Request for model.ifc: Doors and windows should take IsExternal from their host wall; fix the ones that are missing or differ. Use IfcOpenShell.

First a look at what the model holds.

```python
import ifcopenshell
import ifcopenshell.util.element

model = ifcopenshell.open("model.ifc")
print(model.schema)
seen = {}
for e in model.by_type("IfcDoor") + model.by_type("IfcWindow"):
    if not e.FillsVoids:
        continue
    host = e.FillsVoids[0].RelatingOpeningElement.VoidsElements[0].RelatingBuildingElement
    own = ifcopenshell.util.element.get_pset(e, f"Pset_{e.is_a()[3:].removesuffix('StandardCase')}Common", "IsExternal")
    wall = ifcopenshell.util.element.get_pset(host, "Pset_WallCommon", "IsExternal")
    seen[e.is_a(), own, wall] = seen.get((e.is_a(), own, wall), 0) + 1
for (cls, own, wall), count in sorted(seen.items(), key=str):
    print(count, cls, "IsExternal:", own, "| host wall:", wall)
```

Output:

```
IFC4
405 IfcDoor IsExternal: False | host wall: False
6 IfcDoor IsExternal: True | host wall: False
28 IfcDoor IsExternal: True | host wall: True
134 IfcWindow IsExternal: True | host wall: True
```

```python
import ifcopenshell
import ifcopenshell.api.pset
import ifcopenshell.util.element

model = ifcopenshell.open("model.ifc")

count = 0
for ifc_class, pset_name in (("IfcDoor", "Pset_DoorCommon"), ("IfcWindow", "Pset_WindowCommon")):
    for e in model.by_type(ifc_class):
        if not e.FillsVoids:
            continue
        host = e.FillsVoids[0].RelatingOpeningElement.VoidsElements[0].RelatingBuildingElement
        external = ifcopenshell.util.element.get_pset(host, "Pset_WallCommon", "IsExternal")
        if external is None or ifcopenshell.util.element.get_pset(e, pset_name, "IsExternal") == external:
            continue
        pset = ifcopenshell.api.pset.add_pset(model, product=e, name=pset_name)
        ifcopenshell.api.pset.edit_pset(model, pset=pset, properties={"IsExternal": external})
        count += 1

print(count, "updated")

model.write("model_edited.ifc")
```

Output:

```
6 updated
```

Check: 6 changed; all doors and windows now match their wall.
